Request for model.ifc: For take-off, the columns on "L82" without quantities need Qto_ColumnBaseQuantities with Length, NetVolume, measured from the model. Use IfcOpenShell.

First a look at what the model holds.

```python
import ifcopenshell
import ifcopenshell.util.element
import ifcopenshell.util.unit

model = ifcopenshell.open("model.ifc")
print(model.schema)
for unit_type in ("LENGTHUNIT", "AREAUNIT", "VOLUMEUNIT"):
    print(unit_type, ifcopenshell.util.unit.calculate_unit_scale(model, unit_type))
storey = next(s for s in model.by_type("IfcBuildingStorey") if s.Name == "L82")
columns = [e for e in ifcopenshell.util.element.get_decomposition(storey) if e.is_a("IfcColumn")]
for e in sorted(columns, key=lambda e: e.id()):
    print(e.id(), e.is_a(), e.Name, list(ifcopenshell.util.element.get_psets(e, qtos_only=True)), sep=" | ")
```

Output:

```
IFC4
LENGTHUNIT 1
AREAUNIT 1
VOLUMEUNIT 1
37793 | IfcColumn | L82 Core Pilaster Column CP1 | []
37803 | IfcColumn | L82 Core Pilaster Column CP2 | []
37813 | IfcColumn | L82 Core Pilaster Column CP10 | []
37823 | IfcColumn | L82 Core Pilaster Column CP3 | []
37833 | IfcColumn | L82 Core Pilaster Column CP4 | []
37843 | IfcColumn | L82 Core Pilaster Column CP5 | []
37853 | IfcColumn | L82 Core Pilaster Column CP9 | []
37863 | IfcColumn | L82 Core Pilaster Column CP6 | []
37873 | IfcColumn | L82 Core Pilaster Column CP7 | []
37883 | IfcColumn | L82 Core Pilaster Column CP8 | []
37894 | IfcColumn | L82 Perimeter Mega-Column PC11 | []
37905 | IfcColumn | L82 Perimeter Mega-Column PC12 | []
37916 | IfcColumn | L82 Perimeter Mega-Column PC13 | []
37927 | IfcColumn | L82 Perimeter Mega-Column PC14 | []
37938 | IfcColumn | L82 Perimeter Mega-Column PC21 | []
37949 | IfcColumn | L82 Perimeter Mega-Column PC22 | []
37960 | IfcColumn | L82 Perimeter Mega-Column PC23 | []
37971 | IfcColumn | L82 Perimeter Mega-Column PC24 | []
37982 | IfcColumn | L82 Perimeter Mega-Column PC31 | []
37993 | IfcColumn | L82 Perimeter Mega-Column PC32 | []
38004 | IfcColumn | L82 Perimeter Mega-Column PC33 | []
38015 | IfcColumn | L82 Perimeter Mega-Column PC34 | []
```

```python
import ifcopenshell
import ifcopenshell.api.pset
import ifcopenshell.geom
import ifcopenshell.util.element
import ifcopenshell.util.shape
import ifcopenshell.util.unit

model = ifcopenshell.open("model.ifc")
unit_scale = ifcopenshell.util.unit.calculate_unit_scale(model)
volume_scale = ifcopenshell.util.unit.calculate_unit_scale(model, "VOLUMEUNIT")
settings = ifcopenshell.geom.settings()

storey = next(s for s in model.by_type("IfcBuildingStorey") if s.Name == "L82")
columns = [e for e in ifcopenshell.util.element.get_decomposition(storey) if e.is_a("IfcColumn")]

for e in sorted(columns, key=lambda e: e.id()):
    if ifcopenshell.util.element.get_psets(e, qtos_only=True, should_inherit=False):
        continue
    # Geometry comes back in metres, in the element's own axes.
    shape = ifcopenshell.geom.create_shape(settings, e)
    values = {
        "Length": ifcopenshell.util.shape.get_z(shape.geometry) / unit_scale,
        "NetVolume": ifcopenshell.util.shape.get_volume(shape.geometry) / volume_scale,
    }
    qto = ifcopenshell.api.pset.add_qto(model, product=e, name="Qto_ColumnBaseQuantities")
    ifcopenshell.api.pset.edit_qto(model, qto=qto, properties=values)
    print(e.id(), {k: round(v, 3) for k, v in values.items()})

model.write("model-out.ifc")
```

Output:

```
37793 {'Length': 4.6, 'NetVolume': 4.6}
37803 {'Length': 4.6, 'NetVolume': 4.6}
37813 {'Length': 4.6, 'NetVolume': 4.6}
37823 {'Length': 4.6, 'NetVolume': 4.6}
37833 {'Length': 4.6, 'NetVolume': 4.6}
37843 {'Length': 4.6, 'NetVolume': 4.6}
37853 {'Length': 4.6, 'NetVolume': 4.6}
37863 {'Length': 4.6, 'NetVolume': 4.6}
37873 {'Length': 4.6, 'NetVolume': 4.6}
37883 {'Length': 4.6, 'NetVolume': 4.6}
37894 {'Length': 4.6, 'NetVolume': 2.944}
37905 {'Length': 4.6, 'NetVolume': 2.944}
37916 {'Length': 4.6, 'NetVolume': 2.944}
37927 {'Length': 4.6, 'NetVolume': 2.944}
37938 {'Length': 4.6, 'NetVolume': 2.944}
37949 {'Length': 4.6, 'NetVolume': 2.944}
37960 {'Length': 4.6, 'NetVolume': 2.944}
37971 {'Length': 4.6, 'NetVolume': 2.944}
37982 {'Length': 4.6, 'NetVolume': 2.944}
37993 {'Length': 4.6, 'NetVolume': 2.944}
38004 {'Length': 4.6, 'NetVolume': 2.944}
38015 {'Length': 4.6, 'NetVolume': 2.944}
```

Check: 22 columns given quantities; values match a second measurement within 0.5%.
